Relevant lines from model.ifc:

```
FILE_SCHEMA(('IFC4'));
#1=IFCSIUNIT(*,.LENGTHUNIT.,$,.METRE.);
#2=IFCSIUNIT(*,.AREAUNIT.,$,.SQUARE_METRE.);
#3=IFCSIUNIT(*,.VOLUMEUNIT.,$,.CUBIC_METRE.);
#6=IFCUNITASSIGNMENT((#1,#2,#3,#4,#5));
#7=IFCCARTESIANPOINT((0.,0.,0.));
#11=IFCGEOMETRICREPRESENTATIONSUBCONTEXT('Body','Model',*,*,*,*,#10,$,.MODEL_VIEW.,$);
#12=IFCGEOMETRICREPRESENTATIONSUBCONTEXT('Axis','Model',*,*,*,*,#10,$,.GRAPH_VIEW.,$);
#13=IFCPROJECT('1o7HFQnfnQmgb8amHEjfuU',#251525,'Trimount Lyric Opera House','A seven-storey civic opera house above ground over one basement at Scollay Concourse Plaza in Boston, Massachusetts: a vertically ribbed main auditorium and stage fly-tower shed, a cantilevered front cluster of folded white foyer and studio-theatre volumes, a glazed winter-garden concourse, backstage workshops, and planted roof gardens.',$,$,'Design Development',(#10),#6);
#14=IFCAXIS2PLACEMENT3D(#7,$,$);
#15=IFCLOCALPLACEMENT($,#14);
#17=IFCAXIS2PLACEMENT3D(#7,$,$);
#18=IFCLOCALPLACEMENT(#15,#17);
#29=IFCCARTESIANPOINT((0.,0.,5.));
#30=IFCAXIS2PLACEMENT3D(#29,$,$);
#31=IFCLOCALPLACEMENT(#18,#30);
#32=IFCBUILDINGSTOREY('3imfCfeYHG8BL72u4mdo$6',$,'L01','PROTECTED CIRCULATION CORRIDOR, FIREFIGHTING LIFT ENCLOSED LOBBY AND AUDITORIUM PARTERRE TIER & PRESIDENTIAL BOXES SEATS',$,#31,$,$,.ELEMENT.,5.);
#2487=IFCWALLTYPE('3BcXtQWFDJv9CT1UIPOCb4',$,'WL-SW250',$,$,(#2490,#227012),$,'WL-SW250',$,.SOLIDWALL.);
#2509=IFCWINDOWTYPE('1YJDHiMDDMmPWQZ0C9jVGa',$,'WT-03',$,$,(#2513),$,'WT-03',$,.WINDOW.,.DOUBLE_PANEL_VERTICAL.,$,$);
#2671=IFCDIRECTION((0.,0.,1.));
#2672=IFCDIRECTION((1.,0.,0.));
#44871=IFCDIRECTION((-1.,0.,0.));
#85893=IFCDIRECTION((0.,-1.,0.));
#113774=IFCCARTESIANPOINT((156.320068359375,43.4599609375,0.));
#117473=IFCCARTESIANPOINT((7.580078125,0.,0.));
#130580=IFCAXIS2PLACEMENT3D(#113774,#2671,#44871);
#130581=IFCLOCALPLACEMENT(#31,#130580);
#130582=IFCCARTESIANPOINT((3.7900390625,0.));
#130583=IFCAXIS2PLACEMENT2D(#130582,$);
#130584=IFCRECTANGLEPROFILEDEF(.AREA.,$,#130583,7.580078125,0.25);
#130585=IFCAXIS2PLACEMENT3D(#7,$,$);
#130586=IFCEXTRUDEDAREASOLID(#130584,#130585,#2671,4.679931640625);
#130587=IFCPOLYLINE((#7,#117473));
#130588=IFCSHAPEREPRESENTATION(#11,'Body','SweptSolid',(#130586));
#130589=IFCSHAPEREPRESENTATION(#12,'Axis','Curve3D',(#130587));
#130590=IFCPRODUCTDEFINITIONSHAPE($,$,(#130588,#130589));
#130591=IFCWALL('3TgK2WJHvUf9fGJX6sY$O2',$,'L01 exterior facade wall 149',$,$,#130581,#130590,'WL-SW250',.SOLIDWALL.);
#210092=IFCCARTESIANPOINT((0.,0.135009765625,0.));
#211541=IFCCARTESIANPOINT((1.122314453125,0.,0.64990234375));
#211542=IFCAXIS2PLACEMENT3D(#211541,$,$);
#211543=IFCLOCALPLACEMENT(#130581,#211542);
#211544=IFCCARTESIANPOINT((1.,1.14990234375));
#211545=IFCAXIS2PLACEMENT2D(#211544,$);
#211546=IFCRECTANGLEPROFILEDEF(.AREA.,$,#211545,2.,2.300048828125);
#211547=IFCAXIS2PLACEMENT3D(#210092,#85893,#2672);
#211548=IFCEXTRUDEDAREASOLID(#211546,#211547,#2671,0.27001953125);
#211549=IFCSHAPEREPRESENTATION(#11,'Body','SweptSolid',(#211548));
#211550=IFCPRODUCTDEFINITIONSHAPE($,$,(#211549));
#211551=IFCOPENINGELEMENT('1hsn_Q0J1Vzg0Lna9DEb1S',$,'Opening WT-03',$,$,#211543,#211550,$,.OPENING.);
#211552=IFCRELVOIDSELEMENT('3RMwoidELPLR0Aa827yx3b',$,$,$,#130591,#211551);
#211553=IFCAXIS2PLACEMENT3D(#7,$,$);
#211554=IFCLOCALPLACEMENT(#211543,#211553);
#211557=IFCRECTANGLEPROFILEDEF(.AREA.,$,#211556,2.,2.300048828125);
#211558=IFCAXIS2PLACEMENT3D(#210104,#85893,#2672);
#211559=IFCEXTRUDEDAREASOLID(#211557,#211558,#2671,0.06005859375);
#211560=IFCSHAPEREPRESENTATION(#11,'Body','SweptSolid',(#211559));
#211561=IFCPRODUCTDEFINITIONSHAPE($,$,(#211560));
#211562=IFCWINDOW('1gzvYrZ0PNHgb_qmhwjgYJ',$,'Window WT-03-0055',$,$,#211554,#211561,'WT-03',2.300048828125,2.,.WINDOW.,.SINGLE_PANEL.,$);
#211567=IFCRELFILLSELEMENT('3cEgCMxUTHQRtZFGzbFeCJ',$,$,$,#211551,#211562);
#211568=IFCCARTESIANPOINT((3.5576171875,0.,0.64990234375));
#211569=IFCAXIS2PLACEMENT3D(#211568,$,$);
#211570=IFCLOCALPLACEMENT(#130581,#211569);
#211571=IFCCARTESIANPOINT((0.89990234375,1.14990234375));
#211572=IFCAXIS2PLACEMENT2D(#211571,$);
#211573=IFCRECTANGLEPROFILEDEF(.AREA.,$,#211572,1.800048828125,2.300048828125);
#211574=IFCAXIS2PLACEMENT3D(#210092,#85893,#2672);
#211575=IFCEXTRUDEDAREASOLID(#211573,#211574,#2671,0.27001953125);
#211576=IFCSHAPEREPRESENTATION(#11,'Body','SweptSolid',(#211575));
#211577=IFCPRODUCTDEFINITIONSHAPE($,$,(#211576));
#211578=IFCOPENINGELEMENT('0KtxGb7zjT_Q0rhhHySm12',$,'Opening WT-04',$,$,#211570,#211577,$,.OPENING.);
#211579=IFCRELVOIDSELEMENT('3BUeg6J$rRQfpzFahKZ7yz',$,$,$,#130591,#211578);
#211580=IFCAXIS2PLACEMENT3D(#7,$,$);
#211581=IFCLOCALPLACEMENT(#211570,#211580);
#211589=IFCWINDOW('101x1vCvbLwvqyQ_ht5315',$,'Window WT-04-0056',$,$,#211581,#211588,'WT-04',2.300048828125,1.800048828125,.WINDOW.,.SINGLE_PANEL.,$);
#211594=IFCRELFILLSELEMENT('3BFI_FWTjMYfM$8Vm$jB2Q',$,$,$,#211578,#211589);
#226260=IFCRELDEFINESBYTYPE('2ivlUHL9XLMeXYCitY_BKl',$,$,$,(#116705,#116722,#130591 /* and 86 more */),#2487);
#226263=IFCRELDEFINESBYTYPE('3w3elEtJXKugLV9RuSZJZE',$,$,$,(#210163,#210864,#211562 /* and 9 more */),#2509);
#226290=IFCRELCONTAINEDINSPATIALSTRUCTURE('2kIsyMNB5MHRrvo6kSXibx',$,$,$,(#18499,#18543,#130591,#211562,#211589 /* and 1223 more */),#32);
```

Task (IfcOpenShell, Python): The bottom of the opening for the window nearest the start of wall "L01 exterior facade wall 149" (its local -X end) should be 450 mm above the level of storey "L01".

```python
import numpy as np
import ifcopenshell
import ifcopenshell.api.geometry
import ifcopenshell.geom
import ifcopenshell.util.element
import ifcopenshell.util.placement
import ifcopenshell.util.shape
import ifcopenshell.util.unit

model = ifcopenshell.open("model.ifc")
unit_scale = ifcopenshell.util.unit.calculate_unit_scale(model)

window = model.by_id(211562)
opening = window.FillsVoids[0].RelatingOpeningElement
storey = ifcopenshell.util.element.get_container(window, ifc_class="IfcBuildingStorey")
level = ifcopenshell.util.placement.get_local_placement(storey.ObjectPlacement)[2, 3]

# The opening's origin need not be at the sill, so measure its lowest point.
shape = ifcopenshell.geom.create_shape(ifcopenshell.geom.settings(), opening)
bottom = ifcopenshell.util.shape.get_shape_bottom_elevation(shape, shape.geometry) / unit_scale
dz = level + 0.45 / unit_scale - bottom

shift = np.array([0.0, 0.0, dz])
# The window is placed relative to its opening, so it follows when the opening moves.
matrix = ifcopenshell.util.placement.get_local_placement(opening.ObjectPlacement)
matrix[:3, 3] += shift
ifcopenshell.api.geometry.edit_object_placement(
    model, product=opening, matrix=matrix, is_si=False, should_transform_children=True
)

print(f"moved by {dz * unit_scale:+.3f} m")

model.write("model_updated.ifc")
```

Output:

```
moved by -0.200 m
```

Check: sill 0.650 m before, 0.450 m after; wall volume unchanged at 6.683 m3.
